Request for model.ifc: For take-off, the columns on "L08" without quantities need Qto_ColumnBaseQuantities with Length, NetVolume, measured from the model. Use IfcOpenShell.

First a look at what the model holds.

```python
import ifcopenshell
import ifcopenshell.util.element
import ifcopenshell.util.unit

model = ifcopenshell.open("model.ifc")
print(model.schema)
for unit_type in ("LENGTHUNIT", "AREAUNIT", "VOLUMEUNIT"):
    print(unit_type, ifcopenshell.util.unit.calculate_unit_scale(model, unit_type))
storey = next(s for s in model.by_type("IfcBuildingStorey") if s.Name == "L08")
columns = [e for e in ifcopenshell.util.element.get_decomposition(storey) if e.is_a("IfcColumn")]
for e in sorted(columns, key=lambda e: e.id()):
    print(e.id(), e.is_a(), e.Name, list(ifcopenshell.util.element.get_psets(e, qtos_only=True)), sep=" | ")
```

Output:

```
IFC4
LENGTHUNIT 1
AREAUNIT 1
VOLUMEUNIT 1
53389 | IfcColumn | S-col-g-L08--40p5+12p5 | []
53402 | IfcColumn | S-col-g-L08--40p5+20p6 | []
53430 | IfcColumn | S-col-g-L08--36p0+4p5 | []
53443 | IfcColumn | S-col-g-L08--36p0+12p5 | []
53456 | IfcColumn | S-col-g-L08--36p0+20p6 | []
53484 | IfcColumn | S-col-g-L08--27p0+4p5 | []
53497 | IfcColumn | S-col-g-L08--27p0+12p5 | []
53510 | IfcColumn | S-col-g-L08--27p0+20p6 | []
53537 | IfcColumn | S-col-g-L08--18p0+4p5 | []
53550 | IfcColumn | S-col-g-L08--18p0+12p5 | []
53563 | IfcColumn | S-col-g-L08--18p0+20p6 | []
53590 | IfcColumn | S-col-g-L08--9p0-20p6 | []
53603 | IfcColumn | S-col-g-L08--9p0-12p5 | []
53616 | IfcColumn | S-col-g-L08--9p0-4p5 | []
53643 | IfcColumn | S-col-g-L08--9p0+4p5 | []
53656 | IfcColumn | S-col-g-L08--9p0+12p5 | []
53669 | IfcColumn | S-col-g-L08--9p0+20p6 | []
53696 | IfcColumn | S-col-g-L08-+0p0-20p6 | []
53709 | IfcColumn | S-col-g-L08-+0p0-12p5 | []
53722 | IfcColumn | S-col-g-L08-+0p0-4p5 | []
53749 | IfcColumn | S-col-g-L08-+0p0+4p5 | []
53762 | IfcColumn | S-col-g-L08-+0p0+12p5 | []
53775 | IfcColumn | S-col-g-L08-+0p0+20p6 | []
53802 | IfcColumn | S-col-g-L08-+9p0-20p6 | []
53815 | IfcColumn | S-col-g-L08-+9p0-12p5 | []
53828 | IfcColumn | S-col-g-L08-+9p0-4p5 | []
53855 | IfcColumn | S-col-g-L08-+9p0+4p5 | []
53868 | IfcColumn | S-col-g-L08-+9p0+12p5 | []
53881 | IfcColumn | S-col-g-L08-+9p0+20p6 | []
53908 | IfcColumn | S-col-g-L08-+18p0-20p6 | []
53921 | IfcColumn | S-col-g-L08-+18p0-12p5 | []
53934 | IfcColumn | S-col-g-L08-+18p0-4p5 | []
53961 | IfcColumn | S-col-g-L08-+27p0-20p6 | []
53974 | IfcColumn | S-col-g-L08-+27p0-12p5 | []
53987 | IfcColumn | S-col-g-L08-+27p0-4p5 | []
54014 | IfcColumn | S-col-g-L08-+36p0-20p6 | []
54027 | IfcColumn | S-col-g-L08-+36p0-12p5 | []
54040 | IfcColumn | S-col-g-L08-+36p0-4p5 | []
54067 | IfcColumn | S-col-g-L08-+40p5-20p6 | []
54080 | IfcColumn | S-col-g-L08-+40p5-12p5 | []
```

```python
import ifcopenshell
import ifcopenshell.api.pset
import ifcopenshell.geom
import ifcopenshell.util.element
import ifcopenshell.util.shape
import ifcopenshell.util.unit

model = ifcopenshell.open("model.ifc")
unit_scale = ifcopenshell.util.unit.calculate_unit_scale(model)
volume_scale = ifcopenshell.util.unit.calculate_unit_scale(model, "VOLUMEUNIT")
settings = ifcopenshell.geom.settings()

storey = next(s for s in model.by_type("IfcBuildingStorey") if s.Name == "L08")
columns = [e for e in ifcopenshell.util.element.get_decomposition(storey) if e.is_a("IfcColumn")]

for e in sorted(columns, key=lambda e: e.id()):
    if ifcopenshell.util.element.get_psets(e, qtos_only=True, should_inherit=False):
        continue
    # Geometry comes back in metres, in the element's own axes.
    shape = ifcopenshell.geom.create_shape(settings, e)
    values = {
        "Length": ifcopenshell.util.shape.get_z(shape.geometry) / unit_scale,
        "NetVolume": ifcopenshell.util.shape.get_volume(shape.geometry) / volume_scale,
    }
    qto = ifcopenshell.api.pset.add_qto(model, product=e, name="Qto_ColumnBaseQuantities")
    ifcopenshell.api.pset.edit_qto(model, qto=qto, properties=values)
    print(e.id(), {k: round(v, 3) for k, v in values.items()})

model.write("model_v2.ifc")
```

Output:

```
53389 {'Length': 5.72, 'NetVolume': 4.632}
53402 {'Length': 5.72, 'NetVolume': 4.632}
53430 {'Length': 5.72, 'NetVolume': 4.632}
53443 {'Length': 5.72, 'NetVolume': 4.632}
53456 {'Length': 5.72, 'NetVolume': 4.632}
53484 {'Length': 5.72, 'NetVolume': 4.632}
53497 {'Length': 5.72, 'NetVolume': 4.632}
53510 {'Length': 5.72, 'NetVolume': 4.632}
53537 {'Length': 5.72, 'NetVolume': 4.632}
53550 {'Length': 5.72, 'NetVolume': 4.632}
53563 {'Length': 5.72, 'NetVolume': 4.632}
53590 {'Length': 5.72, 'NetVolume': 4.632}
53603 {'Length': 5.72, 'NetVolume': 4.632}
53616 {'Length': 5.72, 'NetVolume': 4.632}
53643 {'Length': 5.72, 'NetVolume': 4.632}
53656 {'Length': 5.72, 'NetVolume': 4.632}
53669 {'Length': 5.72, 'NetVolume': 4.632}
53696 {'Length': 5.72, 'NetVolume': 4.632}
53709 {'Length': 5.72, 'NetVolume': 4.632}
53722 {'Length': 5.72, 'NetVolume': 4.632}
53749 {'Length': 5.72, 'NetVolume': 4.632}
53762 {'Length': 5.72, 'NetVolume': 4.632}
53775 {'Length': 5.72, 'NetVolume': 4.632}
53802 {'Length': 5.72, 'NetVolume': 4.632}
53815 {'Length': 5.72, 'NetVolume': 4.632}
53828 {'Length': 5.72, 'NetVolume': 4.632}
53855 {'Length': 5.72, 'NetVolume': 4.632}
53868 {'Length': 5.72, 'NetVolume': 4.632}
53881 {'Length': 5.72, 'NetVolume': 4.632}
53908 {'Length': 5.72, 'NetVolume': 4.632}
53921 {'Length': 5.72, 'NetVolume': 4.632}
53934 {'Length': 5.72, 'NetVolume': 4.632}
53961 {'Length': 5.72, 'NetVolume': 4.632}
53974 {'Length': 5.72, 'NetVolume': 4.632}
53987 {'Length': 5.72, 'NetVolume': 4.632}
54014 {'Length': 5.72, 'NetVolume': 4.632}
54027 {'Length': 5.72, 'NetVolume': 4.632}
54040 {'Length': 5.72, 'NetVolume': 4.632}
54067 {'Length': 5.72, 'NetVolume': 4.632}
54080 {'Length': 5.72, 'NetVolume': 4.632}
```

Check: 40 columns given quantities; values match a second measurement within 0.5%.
